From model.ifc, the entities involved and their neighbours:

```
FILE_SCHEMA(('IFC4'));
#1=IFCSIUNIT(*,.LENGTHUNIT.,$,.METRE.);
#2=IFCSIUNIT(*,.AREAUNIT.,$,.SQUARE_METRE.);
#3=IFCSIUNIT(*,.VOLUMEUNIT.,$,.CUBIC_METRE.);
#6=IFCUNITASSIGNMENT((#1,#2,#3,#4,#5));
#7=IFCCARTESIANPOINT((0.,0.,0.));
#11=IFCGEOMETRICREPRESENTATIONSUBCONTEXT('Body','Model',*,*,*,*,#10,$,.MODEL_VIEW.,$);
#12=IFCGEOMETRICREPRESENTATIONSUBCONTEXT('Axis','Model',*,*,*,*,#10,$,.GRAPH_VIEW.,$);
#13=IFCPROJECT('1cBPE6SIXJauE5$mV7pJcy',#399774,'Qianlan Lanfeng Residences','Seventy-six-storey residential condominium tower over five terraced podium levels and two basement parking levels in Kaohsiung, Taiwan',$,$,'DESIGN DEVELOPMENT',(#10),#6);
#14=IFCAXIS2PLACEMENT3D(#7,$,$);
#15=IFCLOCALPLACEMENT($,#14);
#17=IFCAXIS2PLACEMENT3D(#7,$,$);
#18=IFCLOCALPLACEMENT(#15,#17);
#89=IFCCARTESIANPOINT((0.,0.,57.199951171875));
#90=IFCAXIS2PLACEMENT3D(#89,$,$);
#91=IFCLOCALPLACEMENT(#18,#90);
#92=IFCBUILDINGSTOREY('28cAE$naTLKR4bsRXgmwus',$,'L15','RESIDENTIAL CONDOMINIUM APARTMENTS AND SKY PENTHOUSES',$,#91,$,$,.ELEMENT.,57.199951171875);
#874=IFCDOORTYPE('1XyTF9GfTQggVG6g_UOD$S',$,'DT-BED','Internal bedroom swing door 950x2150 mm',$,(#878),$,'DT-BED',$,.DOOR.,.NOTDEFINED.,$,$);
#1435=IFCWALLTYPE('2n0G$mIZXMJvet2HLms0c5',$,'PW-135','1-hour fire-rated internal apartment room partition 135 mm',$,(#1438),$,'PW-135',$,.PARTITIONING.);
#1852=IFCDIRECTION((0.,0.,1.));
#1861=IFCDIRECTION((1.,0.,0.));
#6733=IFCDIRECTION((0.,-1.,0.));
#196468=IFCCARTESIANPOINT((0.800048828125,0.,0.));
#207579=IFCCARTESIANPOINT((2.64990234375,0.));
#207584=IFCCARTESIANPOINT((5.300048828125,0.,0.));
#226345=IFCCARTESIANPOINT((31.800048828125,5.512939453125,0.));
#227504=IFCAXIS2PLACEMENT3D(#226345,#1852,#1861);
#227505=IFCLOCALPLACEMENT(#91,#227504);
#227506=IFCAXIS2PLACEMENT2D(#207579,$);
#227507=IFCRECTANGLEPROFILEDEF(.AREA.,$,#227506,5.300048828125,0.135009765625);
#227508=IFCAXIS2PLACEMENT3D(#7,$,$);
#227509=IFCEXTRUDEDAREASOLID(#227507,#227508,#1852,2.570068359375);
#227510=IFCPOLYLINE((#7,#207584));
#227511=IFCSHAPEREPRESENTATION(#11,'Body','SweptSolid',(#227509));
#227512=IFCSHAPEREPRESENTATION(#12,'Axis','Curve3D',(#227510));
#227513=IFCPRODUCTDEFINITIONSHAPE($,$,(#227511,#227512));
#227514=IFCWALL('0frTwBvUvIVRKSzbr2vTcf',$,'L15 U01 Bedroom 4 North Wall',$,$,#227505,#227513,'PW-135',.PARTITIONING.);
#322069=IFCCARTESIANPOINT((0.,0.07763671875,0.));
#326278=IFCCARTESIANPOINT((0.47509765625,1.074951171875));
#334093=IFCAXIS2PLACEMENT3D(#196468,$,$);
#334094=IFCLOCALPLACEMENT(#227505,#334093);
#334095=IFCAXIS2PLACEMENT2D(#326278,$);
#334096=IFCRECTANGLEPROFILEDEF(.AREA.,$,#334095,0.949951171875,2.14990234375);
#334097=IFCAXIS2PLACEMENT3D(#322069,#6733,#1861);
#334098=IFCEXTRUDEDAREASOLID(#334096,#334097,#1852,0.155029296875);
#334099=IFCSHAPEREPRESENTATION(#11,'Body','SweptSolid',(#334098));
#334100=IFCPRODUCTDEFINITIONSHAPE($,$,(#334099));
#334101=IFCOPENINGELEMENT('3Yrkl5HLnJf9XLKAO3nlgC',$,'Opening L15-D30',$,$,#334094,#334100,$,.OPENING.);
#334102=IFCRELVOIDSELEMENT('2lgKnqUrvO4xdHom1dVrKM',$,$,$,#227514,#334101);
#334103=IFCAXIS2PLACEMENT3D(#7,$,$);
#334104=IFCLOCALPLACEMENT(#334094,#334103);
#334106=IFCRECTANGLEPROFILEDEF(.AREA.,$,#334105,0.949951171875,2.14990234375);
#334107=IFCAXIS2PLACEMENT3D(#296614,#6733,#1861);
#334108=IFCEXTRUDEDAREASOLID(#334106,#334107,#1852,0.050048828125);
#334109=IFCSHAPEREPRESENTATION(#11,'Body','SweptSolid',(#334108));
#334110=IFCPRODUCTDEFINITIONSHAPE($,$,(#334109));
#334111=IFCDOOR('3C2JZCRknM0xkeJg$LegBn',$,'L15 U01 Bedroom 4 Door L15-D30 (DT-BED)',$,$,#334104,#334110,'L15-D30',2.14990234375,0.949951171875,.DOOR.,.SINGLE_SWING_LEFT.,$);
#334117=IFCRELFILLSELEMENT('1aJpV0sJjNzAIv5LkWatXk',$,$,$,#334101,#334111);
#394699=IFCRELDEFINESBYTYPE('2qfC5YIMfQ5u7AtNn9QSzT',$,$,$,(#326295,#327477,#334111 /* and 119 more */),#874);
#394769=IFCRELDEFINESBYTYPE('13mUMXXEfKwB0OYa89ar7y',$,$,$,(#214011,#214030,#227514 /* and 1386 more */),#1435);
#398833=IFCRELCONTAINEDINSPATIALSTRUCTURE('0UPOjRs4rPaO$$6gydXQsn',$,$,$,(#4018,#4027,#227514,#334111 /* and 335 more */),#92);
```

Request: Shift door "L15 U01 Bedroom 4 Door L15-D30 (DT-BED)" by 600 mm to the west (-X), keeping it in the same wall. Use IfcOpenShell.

```python
import ifcopenshell
import ifcopenshell.api.geometry
import ifcopenshell.util.placement

model = ifcopenshell.open("model.ifc")

door = model.by_guid("3C2JZCRknM0xkeJg$LegBn")
opening = door.FillsVoids[0].RelatingOpeningElement
wall = opening.VoidsElements[0].RelatingBuildingElement

wall_matrix = ifcopenshell.util.placement.get_local_placement(wall.ObjectPlacement)
shift = wall_matrix[:3, 0] * -0.6
before = ifcopenshell.util.placement.get_local_placement(door.ObjectPlacement)[:3, 3].copy()

# The door is placed relative to its opening, so it follows when the opening moves.
matrix = ifcopenshell.util.placement.get_local_placement(opening.ObjectPlacement)
matrix[:3, 3] += shift
ifcopenshell.api.geometry.edit_object_placement(
    model, product=opening, matrix=matrix, is_si=False, should_transform_children=True
)

after = ifcopenshell.util.placement.get_local_placement(door.ObjectPlacement)[:3, 3]
print("door moved by", (after - before).round(3) + 0.0)

model.write("model-out.ifc")
```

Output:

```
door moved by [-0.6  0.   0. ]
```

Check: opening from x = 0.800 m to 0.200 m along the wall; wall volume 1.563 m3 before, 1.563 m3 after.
